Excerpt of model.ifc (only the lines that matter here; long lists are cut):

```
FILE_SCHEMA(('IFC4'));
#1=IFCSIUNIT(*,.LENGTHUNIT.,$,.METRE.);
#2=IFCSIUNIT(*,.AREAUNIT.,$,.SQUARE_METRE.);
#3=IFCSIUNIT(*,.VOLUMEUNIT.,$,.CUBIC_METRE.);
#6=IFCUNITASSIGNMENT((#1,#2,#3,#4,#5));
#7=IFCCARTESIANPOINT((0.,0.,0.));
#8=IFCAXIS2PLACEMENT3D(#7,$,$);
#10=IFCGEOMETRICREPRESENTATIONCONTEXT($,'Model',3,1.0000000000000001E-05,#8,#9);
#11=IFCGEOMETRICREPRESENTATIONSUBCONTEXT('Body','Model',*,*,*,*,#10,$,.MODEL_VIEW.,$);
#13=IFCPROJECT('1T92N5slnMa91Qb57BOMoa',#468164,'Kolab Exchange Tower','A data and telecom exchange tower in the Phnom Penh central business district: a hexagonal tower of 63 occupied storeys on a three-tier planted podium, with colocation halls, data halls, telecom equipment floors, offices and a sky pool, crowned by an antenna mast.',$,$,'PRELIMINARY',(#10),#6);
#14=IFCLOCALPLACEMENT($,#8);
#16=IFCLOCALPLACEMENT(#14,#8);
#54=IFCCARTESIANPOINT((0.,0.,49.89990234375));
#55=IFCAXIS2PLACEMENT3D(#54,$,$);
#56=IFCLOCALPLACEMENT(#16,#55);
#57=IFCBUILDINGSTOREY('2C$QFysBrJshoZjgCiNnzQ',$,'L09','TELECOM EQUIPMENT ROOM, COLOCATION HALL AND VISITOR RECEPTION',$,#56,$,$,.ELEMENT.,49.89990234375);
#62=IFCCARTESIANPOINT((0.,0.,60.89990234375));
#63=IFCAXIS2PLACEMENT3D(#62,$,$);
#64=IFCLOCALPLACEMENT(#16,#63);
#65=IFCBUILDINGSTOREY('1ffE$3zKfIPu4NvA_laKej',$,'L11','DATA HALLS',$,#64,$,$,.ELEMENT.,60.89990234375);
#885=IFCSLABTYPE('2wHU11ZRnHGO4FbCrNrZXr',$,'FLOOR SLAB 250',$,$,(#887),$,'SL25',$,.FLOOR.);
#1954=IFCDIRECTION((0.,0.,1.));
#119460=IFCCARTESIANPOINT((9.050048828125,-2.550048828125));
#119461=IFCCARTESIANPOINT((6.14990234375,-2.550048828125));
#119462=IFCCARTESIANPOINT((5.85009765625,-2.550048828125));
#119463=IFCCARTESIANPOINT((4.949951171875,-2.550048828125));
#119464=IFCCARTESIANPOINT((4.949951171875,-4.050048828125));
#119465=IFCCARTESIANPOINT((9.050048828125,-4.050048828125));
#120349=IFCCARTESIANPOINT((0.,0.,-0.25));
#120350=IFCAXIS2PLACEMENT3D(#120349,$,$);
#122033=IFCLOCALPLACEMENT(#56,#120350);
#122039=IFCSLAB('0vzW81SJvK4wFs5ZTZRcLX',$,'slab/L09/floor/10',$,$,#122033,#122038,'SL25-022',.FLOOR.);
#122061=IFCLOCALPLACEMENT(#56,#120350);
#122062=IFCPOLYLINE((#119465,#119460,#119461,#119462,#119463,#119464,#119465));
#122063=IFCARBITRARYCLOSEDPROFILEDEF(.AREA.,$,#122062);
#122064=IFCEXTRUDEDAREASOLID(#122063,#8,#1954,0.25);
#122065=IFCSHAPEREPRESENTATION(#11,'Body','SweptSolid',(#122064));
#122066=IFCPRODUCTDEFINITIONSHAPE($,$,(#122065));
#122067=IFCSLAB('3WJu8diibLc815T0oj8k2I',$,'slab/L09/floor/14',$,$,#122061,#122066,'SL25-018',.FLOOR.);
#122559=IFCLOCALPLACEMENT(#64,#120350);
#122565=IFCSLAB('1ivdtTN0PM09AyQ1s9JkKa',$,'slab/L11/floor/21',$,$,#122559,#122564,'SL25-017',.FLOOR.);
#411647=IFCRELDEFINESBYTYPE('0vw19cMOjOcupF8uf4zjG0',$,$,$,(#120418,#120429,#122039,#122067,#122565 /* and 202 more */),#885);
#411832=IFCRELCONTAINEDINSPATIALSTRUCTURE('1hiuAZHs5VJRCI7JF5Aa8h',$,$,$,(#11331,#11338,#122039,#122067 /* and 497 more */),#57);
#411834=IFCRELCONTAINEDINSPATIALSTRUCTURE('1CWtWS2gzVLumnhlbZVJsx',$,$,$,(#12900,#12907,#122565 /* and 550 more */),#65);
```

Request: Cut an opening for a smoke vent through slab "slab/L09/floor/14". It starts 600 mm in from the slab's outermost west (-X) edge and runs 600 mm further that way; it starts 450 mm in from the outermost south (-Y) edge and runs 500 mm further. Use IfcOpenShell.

```python
import numpy as np
import ifcopenshell
import ifcopenshell.api.feature
import ifcopenshell.api.geometry
import ifcopenshell.api.root
import ifcopenshell.geom
import ifcopenshell.util.placement
import ifcopenshell.util.representation
import ifcopenshell.util.shape
import ifcopenshell.util.unit

model = ifcopenshell.open("model.ifc")
unit_scale = ifcopenshell.util.unit.calculate_unit_scale(model)
settings = ifcopenshell.geom.settings()


def volume(element):
    """Net volume in cubic metres, openings subtracted."""
    shape = ifcopenshell.geom.create_shape(settings, element)
    return ifcopenshell.util.shape.get_volume(shape.geometry)


slab = model.by_guid("3WJu8diibLc815T0oj8k2I")
before = volume(slab)

# Extent in the slab's own axes, in metres. The edges named are its -X and -Y sides.
slab_shape = ifcopenshell.geom.create_shape(settings, slab)
vertices = ifcopenshell.util.shape.get_vertices(slab_shape.geometry)
x_min, y_min, bottom = vertices.min(axis=0)
top = vertices[:, 2].max()

opening = ifcopenshell.api.root.create_entity(model, ifc_class="IfcOpeningElement", name="Smoke vent opening", predefined_type="OPENING")
context = ifcopenshell.util.representation.get_context(model, "Model", "Body", "MODEL_VIEW")
width, depth = 0.6, 0.5
outline = [(0.0, 0.0), (width, 0.0), (width, depth), (0.0, depth), (0.0, 0.0)]
# Overshoot both faces by 50 mm so the cut is clean.
shape = ifcopenshell.api.geometry.add_slab_representation(
    model, context=context, depth=top - bottom + 0.1, polyline=outline
)
ifcopenshell.api.geometry.assign_representation(model, product=opening, representation=shape)

matrix = ifcopenshell.util.placement.get_local_placement(slab.ObjectPlacement)
matrix[:, 3] = matrix @ np.append(np.array([x_min + 0.6, y_min + 0.45, bottom - 0.05]) / unit_scale, 1.0)
ifcopenshell.api.geometry.edit_object_placement(model, product=opening, matrix=matrix, is_si=False)
ifcopenshell.api.feature.add_feature(model, feature=opening, element=slab)

after = volume(slab)

print(f"slab volume {before:.3f} -> {after:.3f} m3")

model.write("model_rev.ifc")
```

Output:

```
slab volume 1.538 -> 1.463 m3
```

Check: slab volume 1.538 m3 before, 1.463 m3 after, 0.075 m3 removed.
